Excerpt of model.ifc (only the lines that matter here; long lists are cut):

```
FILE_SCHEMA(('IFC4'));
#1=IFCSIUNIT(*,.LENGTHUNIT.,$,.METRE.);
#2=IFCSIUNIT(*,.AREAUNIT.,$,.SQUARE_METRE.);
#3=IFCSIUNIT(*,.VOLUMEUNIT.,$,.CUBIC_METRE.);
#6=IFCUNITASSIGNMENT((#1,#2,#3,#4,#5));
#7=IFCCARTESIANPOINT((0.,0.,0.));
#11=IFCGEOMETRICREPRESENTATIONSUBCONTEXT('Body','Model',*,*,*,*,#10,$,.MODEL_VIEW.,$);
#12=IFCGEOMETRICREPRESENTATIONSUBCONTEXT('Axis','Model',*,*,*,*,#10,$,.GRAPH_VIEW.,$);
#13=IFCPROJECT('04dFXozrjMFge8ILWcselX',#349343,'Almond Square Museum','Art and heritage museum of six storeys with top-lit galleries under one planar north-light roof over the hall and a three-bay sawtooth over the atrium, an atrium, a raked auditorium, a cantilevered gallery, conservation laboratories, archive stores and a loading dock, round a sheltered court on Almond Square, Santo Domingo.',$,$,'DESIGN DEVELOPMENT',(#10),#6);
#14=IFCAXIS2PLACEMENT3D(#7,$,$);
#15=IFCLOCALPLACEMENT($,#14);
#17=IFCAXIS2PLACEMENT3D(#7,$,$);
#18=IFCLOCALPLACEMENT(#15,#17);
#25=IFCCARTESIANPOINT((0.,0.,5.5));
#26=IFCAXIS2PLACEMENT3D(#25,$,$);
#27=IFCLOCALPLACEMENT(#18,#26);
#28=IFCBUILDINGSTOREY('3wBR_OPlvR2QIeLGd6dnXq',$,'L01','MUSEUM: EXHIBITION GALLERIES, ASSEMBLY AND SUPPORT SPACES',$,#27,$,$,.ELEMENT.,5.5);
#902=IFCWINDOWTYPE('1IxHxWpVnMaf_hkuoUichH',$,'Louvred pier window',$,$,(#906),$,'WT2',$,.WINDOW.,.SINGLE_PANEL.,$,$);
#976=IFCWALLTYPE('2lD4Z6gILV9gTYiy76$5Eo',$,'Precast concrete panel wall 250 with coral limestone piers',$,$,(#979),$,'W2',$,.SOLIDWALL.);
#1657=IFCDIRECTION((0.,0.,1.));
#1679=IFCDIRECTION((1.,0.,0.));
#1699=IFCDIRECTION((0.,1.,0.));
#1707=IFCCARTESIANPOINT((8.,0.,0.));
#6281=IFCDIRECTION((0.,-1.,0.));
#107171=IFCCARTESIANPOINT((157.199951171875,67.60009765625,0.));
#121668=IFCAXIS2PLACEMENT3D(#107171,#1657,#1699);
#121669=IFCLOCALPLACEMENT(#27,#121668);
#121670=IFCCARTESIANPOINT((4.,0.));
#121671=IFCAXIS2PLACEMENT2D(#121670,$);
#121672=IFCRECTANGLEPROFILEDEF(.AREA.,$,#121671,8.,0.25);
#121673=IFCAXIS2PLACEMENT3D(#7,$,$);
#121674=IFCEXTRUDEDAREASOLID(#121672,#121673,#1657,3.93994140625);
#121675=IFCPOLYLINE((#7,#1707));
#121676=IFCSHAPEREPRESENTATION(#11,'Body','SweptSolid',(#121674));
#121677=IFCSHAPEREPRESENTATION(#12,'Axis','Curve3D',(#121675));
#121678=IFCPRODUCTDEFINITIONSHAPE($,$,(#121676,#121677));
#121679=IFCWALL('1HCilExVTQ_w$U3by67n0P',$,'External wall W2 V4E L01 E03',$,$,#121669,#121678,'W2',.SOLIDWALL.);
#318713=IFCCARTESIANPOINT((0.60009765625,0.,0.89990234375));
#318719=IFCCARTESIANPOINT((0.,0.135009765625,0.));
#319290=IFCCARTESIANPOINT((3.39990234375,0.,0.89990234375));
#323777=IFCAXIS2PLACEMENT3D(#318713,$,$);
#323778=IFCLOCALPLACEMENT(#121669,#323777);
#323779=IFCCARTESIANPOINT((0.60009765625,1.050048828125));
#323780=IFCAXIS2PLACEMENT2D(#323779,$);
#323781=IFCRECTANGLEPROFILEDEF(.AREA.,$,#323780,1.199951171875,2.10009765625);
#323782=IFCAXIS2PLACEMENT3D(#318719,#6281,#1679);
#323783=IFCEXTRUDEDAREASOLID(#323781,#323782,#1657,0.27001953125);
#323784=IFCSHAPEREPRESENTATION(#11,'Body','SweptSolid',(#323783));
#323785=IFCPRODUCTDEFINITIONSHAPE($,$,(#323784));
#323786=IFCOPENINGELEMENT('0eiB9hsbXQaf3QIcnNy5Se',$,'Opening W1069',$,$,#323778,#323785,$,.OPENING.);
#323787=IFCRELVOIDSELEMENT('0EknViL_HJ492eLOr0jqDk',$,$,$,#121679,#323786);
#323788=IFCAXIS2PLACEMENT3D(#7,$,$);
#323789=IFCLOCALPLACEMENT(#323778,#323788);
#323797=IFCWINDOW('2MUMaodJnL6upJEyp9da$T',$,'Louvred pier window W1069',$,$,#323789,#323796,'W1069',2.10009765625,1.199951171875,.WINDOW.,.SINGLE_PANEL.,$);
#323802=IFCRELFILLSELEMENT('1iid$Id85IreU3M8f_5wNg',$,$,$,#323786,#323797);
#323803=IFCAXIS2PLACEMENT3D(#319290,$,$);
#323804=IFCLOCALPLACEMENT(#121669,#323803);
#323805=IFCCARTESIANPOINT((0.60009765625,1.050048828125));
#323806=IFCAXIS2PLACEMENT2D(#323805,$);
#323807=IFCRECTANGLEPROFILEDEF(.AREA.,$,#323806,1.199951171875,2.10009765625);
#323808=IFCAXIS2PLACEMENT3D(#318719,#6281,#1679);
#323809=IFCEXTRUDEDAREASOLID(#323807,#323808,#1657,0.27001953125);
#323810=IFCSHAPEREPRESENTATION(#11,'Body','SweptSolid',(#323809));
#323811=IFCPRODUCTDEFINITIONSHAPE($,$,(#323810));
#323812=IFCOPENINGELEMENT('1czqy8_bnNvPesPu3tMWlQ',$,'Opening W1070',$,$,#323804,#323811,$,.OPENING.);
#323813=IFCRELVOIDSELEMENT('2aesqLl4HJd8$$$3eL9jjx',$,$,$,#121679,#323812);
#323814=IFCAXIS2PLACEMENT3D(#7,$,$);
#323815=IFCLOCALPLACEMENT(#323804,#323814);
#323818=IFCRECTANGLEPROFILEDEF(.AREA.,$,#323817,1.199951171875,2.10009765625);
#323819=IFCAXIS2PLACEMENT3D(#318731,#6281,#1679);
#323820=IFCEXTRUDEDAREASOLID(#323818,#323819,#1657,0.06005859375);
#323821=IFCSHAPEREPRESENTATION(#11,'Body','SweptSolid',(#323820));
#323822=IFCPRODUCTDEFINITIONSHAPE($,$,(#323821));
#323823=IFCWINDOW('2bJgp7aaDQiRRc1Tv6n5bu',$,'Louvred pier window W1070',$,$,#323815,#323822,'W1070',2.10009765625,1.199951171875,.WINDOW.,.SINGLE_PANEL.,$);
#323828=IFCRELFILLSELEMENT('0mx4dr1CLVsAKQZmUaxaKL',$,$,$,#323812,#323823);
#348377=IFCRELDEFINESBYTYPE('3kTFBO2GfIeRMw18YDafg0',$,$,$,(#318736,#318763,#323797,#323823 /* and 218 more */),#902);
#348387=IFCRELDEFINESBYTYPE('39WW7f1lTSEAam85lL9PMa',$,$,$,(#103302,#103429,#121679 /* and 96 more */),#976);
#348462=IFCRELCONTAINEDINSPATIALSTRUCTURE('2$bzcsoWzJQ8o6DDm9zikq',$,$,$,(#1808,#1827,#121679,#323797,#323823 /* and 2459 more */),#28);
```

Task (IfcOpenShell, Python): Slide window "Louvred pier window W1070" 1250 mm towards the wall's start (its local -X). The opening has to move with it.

```python
import ifcopenshell
import ifcopenshell.api.geometry
import ifcopenshell.util.placement

model = ifcopenshell.open("model.ifc")

window = model.by_guid("2bJgp7aaDQiRRc1Tv6n5bu")
opening = window.FillsVoids[0].RelatingOpeningElement
wall = opening.VoidsElements[0].RelatingBuildingElement

wall_matrix = ifcopenshell.util.placement.get_local_placement(wall.ObjectPlacement)
shift = wall_matrix[:3, 0] * -1.25
before = ifcopenshell.util.placement.get_local_placement(window.ObjectPlacement)[:3, 3].copy()

# The window is placed relative to its opening, so it follows when the opening moves.
matrix = ifcopenshell.util.placement.get_local_placement(opening.ObjectPlacement)
matrix[:3, 3] += shift
ifcopenshell.api.geometry.edit_object_placement(
    model, product=opening, matrix=matrix, is_si=False, should_transform_children=True
)

after = ifcopenshell.util.placement.get_local_placement(window.ObjectPlacement)[:3, 3]
print("window moved by", (after - before).round(3) + 0.0)

model.write("model-out.ifc")
```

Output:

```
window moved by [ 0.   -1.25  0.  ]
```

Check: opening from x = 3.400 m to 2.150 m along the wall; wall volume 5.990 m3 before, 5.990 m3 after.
